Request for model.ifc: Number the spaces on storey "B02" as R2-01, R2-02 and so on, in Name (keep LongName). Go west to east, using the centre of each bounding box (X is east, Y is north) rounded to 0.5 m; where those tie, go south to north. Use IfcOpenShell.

First a look at what the model holds.

```python
import ifcopenshell
import ifcopenshell.util.element
import ifcopenshell.util.placement

model = ifcopenshell.open("model.ifc")
print(model.schema)
storey = next(s for s in model.by_type("IfcBuildingStorey") if s.Name == "B02")
spaces = [e for e in ifcopenshell.util.element.get_decomposition(storey) if e.is_a("IfcSpace")]
for e in sorted(spaces, key=lambda e: e.id()):
    origin = ifcopenshell.util.placement.get_local_placement(e.ObjectPlacement)[:3, 3]
    print(e.id(), e.Name, e.LongName, origin.round(2) + 0.0, sep=" | ")
```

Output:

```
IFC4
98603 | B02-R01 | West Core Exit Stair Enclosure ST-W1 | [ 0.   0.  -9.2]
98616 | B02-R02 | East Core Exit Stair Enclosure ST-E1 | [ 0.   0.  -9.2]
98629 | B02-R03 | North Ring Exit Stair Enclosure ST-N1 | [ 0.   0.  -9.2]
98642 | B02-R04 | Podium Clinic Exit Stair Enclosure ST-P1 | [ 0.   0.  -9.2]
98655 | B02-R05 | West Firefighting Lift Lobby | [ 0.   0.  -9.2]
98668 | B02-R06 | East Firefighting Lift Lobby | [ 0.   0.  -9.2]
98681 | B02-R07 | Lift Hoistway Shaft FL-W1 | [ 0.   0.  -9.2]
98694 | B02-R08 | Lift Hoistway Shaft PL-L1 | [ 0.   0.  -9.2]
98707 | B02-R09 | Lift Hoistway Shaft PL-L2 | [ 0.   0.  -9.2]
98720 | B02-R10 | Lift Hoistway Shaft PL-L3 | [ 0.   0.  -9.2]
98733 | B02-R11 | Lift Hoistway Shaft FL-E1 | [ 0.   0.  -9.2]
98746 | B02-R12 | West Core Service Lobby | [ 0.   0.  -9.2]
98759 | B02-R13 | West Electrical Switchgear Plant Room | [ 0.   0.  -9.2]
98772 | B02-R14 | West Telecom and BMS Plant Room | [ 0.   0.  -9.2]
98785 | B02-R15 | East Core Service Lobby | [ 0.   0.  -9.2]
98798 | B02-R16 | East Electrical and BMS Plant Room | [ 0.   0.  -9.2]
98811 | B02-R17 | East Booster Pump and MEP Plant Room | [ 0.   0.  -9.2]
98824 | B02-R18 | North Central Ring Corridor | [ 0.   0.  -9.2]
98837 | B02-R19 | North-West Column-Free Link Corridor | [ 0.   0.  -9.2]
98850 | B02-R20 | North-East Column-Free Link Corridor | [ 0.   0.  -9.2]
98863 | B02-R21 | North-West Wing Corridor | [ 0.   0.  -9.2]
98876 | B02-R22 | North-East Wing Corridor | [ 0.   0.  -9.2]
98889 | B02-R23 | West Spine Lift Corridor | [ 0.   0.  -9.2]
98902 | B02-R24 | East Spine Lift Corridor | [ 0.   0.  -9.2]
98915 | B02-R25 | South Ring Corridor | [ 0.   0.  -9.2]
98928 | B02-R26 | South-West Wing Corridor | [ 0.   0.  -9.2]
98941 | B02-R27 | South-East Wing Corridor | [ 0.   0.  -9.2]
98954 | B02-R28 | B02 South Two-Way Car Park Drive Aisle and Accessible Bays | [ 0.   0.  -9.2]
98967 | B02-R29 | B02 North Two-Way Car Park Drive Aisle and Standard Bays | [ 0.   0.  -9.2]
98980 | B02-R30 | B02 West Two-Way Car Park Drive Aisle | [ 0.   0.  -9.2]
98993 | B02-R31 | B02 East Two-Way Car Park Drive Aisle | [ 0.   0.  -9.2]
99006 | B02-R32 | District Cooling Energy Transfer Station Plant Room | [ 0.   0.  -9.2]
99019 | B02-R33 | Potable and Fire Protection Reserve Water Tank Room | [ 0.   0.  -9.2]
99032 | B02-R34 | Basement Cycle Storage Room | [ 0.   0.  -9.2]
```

```python
import ifcopenshell
import ifcopenshell.geom
import ifcopenshell.util.element
import ifcopenshell.util.shape

model = ifcopenshell.open("model.ifc")
settings = ifcopenshell.geom.settings()
settings.set("use-world-coords", True)


def centre(element):
    shape = ifcopenshell.geom.create_shape(settings, element)
    return ifcopenshell.util.shape.get_bbox_centroid(shape.geometry)


storey = next(s for s in model.by_type("IfcBuildingStorey") if s.Name == "B02")
spaces = [e for e in ifcopenshell.util.element.get_decomposition(storey) if e.is_a("IfcSpace")]

# Insertion points can sit at a corner or the storey origin, so sort by the geometry (in metres).
centres = {e: centre(e) for e in spaces}
spaces.sort(key=lambda e: (round(centres[e][0] / 0.5), centres[e][1]))

for i, e in enumerate(spaces, start=1):
    number = f"R2-{i:02d}"
    e.Name = number
    print(e.id(), number)

model.write("model-out.ifc")
```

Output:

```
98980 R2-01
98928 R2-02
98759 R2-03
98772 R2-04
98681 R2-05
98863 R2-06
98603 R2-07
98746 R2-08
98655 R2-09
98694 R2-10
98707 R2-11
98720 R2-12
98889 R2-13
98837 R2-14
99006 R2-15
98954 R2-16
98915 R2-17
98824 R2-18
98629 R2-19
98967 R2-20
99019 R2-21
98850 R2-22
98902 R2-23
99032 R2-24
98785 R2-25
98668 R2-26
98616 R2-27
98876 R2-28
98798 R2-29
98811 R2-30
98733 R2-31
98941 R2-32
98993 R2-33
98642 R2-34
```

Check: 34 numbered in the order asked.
